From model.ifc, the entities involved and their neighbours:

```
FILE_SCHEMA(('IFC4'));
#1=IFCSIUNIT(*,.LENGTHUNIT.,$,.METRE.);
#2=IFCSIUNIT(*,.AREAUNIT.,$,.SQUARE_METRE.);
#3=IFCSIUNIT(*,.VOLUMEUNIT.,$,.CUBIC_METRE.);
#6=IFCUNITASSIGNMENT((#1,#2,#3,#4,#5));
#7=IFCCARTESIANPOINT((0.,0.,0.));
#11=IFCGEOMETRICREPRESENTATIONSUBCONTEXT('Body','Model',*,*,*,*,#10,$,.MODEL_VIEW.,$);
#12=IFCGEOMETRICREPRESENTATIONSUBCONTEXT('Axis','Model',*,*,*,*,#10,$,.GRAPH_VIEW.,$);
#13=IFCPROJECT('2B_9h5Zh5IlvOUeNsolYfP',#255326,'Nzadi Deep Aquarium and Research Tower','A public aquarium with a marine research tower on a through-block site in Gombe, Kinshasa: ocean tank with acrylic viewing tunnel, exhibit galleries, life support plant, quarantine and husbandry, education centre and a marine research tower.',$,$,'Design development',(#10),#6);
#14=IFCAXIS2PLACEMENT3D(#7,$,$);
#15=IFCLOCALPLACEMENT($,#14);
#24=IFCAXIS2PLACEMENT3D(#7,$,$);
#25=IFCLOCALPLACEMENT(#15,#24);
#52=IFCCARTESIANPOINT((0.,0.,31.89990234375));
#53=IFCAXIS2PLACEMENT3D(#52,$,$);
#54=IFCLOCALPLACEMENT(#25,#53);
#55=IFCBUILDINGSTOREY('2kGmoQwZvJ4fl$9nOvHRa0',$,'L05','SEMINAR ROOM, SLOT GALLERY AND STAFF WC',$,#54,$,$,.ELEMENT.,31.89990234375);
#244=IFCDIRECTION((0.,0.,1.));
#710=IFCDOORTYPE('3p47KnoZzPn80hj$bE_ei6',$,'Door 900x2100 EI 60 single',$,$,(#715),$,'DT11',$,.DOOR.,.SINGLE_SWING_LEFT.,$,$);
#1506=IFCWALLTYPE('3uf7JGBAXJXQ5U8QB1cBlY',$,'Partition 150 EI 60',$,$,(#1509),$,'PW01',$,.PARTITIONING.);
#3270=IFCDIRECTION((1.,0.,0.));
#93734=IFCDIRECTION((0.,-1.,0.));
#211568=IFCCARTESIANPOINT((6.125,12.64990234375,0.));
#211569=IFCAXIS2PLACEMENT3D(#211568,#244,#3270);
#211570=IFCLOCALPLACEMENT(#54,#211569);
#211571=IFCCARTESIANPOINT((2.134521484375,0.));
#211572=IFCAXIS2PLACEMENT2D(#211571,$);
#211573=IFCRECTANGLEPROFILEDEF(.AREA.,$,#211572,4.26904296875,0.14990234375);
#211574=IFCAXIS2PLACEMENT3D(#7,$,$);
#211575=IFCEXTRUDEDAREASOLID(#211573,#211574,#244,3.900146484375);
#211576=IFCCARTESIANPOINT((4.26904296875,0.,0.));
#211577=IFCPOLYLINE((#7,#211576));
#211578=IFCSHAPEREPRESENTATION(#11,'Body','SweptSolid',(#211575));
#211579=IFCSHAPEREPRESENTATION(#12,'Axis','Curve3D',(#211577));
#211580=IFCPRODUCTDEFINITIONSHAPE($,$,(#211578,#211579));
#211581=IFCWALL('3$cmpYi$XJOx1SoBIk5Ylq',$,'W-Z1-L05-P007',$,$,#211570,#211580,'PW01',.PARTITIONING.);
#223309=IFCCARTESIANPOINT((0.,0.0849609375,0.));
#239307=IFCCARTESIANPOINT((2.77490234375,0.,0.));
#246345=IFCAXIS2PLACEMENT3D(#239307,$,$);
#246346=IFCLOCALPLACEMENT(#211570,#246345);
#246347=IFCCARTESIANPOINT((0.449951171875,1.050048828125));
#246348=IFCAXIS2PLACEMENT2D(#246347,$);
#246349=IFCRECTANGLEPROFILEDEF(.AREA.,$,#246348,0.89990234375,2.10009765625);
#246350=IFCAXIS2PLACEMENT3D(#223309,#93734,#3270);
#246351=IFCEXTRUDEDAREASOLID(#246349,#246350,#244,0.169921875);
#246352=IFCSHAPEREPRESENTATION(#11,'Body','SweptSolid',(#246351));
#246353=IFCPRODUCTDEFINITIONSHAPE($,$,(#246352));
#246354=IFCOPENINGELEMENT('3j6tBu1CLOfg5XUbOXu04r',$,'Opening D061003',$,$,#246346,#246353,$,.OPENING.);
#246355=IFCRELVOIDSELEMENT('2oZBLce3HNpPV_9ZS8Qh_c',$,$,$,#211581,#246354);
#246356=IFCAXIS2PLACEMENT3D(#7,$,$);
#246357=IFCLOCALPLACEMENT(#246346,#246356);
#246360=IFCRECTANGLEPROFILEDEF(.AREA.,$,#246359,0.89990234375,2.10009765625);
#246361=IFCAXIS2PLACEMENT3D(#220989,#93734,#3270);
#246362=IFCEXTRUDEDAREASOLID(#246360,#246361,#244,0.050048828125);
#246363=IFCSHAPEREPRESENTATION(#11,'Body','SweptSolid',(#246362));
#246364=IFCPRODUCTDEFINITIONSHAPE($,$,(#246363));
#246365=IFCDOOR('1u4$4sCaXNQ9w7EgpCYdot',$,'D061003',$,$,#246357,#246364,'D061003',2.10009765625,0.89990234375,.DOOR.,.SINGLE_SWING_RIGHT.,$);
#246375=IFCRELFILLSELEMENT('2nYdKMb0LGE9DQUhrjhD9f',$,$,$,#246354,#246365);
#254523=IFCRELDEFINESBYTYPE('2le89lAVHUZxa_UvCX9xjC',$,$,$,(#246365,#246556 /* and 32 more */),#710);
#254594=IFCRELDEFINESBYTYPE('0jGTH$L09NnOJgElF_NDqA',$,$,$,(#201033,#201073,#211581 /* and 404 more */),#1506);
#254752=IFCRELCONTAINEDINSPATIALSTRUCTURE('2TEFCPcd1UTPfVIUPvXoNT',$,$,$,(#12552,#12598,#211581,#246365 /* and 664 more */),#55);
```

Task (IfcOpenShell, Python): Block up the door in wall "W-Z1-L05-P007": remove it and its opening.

```python
import ifcopenshell
import ifcopenshell.api.feature
import ifcopenshell.api.root
import ifcopenshell.geom
import ifcopenshell.util.shape

model = ifcopenshell.open("model.ifc")
settings = ifcopenshell.geom.settings()


def volume(element):
    """Net volume in cubic metres, openings subtracted."""
    shape = ifcopenshell.geom.create_shape(settings, element)
    return ifcopenshell.util.shape.get_volume(shape.geometry)


door = model.by_id(246365)
opening = door.FillsVoids[0].RelatingOpeningElement
wall = opening.VoidsElements[0].RelatingBuildingElement
before = volume(wall)

ifcopenshell.api.root.remove_product(model, product=door)
ifcopenshell.api.feature.remove_feature(model, feature=opening)

after = volume(wall)

print(f"wall volume {before:.3f} -> {after:.3f} m3")

model.write("model_updated.ifc")
```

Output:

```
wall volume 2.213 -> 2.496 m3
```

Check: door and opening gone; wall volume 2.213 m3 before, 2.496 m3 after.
